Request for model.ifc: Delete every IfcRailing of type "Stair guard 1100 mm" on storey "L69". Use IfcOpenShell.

First a look at what the model holds.

```python
import ifcopenshell
import ifcopenshell.util.element

model = ifcopenshell.open("model.ifc")
print(model.schema)
storey = next(s for s in model.by_type("IfcBuildingStorey") if s.Name == "L69")
railings = [e for e in ifcopenshell.util.element.get_decomposition(storey) if e.is_a("IfcRailing")]
seen = {}
for e in railings:
    element_type = ifcopenshell.util.element.get_type(e)
    name = element_type.Name if element_type not in (None, e) else None
    seen[name] = seen.get(name, 0) + 1
for name, count in sorted(seen.items(), key=str):
    print(count, "x", name)
```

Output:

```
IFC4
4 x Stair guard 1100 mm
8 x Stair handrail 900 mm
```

```python
import ifcopenshell
import ifcopenshell.api.root
import ifcopenshell.util.element

model = ifcopenshell.open("model.ifc")

storey = next(s for s in model.by_type("IfcBuildingStorey") if s.Name == "L69")
railings = [e for e in ifcopenshell.util.element.get_decomposition(storey) if e.is_a("IfcRailing")]
targets = [e for e in railings if (t := ifcopenshell.util.element.get_type(e)) not in (None, e) and t.Name == "Stair guard 1100 mm"]

for e in targets:
    ifcopenshell.api.root.remove_product(model, product=e)
print(len(targets), "removed")

model.write("model_edited.ifc")
```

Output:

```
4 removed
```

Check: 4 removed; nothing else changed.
